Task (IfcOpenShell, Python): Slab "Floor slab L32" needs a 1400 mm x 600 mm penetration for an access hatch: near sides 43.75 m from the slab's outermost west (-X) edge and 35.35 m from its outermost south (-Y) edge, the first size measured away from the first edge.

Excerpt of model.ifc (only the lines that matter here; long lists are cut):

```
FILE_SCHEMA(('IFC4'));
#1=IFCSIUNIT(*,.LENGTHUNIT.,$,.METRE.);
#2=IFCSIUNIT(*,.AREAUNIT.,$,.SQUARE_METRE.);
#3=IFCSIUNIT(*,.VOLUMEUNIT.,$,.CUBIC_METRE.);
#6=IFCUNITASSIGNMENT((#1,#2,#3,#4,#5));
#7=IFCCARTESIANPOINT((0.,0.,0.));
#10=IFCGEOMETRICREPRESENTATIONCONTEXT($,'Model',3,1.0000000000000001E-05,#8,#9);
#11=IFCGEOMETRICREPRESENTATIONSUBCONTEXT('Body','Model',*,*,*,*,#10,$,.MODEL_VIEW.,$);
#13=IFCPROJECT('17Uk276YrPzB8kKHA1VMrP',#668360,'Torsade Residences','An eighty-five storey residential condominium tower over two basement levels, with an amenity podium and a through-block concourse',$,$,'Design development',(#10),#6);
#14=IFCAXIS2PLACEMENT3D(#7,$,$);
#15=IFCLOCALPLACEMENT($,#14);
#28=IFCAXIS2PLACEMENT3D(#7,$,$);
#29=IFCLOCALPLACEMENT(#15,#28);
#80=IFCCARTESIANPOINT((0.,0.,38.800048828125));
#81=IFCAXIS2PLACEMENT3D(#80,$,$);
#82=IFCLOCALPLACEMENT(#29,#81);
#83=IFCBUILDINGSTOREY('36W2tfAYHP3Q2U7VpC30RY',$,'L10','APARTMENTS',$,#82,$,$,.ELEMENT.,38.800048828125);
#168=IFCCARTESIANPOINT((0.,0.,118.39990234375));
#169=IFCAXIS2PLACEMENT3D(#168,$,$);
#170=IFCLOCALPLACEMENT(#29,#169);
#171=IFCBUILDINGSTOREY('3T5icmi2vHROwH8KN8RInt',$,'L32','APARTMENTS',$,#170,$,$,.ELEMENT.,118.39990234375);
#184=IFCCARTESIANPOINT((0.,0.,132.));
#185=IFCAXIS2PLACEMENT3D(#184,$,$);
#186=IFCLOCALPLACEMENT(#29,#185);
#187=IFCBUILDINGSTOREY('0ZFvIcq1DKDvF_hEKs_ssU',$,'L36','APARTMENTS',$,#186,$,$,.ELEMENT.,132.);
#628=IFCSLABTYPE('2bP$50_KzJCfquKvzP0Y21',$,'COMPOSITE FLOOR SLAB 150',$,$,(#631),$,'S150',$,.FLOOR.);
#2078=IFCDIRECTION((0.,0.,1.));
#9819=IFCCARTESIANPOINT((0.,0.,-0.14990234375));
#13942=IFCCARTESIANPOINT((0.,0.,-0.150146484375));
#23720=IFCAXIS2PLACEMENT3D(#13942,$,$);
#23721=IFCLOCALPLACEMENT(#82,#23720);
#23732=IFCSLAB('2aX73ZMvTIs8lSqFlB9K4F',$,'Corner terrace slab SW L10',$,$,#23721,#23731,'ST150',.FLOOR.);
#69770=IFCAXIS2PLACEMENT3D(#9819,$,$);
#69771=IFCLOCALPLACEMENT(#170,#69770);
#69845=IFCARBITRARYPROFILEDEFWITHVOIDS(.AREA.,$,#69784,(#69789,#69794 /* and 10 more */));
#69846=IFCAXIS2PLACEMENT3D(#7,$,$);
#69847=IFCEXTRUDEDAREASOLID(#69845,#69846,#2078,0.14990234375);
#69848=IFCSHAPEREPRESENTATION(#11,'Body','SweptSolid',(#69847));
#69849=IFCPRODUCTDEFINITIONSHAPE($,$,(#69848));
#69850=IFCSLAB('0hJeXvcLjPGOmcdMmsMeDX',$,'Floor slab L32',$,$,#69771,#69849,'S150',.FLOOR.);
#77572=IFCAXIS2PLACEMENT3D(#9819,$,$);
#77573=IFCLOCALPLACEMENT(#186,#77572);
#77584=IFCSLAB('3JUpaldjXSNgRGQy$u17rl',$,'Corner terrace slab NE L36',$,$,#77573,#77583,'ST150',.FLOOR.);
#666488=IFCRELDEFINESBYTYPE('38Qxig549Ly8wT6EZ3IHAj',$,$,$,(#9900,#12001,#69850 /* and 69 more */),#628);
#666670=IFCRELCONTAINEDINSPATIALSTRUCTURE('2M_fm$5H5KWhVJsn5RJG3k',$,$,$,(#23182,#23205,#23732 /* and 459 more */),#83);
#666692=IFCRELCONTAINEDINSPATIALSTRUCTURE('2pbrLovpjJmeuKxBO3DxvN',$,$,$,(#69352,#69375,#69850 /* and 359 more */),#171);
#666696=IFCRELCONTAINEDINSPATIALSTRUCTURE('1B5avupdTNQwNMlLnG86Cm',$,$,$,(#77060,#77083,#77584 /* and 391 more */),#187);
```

```python
import numpy as np
import ifcopenshell
import ifcopenshell.api.feature
import ifcopenshell.api.geometry
import ifcopenshell.api.root
import ifcopenshell.geom
import ifcopenshell.util.placement
import ifcopenshell.util.representation
import ifcopenshell.util.shape
import ifcopenshell.util.unit

model = ifcopenshell.open("model.ifc")
unit_scale = ifcopenshell.util.unit.calculate_unit_scale(model)
settings = ifcopenshell.geom.settings()


def volume(element):
    """Net volume in cubic metres, openings subtracted."""
    shape = ifcopenshell.geom.create_shape(settings, element)
    return ifcopenshell.util.shape.get_volume(shape.geometry)


slab = model.by_id(69850)
before = volume(slab)

# Extent in the slab's own axes, in metres. The edges named are its -X and -Y sides.
slab_shape = ifcopenshell.geom.create_shape(settings, slab)
vertices = ifcopenshell.util.shape.get_vertices(slab_shape.geometry)
x_min, y_min, bottom = vertices.min(axis=0)
top = vertices[:, 2].max()

opening = ifcopenshell.api.root.create_entity(model, ifc_class="IfcOpeningElement", name="Access hatch opening", predefined_type="OPENING")
context = ifcopenshell.util.representation.get_context(model, "Model", "Body", "MODEL_VIEW")
width, depth = 1.4, 0.6
outline = [(0.0, 0.0), (width, 0.0), (width, depth), (0.0, depth), (0.0, 0.0)]
# Overshoot both faces by 50 mm so the cut is clean.
shape = ifcopenshell.api.geometry.add_slab_representation(
    model, context=context, depth=top - bottom + 0.1, polyline=outline
)
ifcopenshell.api.geometry.assign_representation(model, product=opening, representation=shape)

matrix = ifcopenshell.util.placement.get_local_placement(slab.ObjectPlacement)
matrix[:, 3] = matrix @ np.append(np.array([x_min + 43.75, y_min + 35.35, bottom - 0.05]) / unit_scale, 1.0)
ifcopenshell.api.geometry.edit_object_placement(model, product=opening, matrix=matrix, is_si=False)
ifcopenshell.api.feature.add_feature(model, feature=opening, element=slab)

after = volume(slab)

print(f"slab volume {before:.3f} -> {after:.3f} m3")

model.write("model-out.ifc")
```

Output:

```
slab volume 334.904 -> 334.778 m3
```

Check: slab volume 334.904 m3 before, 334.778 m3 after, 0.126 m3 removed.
